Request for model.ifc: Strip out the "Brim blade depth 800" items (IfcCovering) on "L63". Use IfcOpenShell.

First a look at what the model holds.

```python
import ifcopenshell
import ifcopenshell.util.element

model = ifcopenshell.open("model.ifc")
print(model.schema)
storey = next(s for s in model.by_type("IfcBuildingStorey") if s.Name == "L63")
coverings = [e for e in ifcopenshell.util.element.get_decomposition(storey) if e.is_a("IfcCovering")]
seen = {}
for e in coverings:
    element_type = ifcopenshell.util.element.get_type(e)
    name = element_type.Name if element_type not in (None, e) else None
    seen[name] = seen.get(name, 0) + 1
for name, count in sorted(seen.items(), key=str):
    print(count, "x", name)
```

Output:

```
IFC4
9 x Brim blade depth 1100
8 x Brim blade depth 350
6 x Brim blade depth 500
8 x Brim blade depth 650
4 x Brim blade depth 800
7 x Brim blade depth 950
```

```python
import ifcopenshell
import ifcopenshell.api.root
import ifcopenshell.util.element

model = ifcopenshell.open("model.ifc")

storey = next(s for s in model.by_type("IfcBuildingStorey") if s.Name == "L63")
coverings = [e for e in ifcopenshell.util.element.get_decomposition(storey) if e.is_a("IfcCovering")]
targets = [e for e in coverings if (t := ifcopenshell.util.element.get_type(e)) not in (None, e) and t.Name == "Brim blade depth 800"]

for e in targets:
    ifcopenshell.api.root.remove_product(model, product=e)
print(len(targets), "removed")

model.write("model_updated.ifc")
```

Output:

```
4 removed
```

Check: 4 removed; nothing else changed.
